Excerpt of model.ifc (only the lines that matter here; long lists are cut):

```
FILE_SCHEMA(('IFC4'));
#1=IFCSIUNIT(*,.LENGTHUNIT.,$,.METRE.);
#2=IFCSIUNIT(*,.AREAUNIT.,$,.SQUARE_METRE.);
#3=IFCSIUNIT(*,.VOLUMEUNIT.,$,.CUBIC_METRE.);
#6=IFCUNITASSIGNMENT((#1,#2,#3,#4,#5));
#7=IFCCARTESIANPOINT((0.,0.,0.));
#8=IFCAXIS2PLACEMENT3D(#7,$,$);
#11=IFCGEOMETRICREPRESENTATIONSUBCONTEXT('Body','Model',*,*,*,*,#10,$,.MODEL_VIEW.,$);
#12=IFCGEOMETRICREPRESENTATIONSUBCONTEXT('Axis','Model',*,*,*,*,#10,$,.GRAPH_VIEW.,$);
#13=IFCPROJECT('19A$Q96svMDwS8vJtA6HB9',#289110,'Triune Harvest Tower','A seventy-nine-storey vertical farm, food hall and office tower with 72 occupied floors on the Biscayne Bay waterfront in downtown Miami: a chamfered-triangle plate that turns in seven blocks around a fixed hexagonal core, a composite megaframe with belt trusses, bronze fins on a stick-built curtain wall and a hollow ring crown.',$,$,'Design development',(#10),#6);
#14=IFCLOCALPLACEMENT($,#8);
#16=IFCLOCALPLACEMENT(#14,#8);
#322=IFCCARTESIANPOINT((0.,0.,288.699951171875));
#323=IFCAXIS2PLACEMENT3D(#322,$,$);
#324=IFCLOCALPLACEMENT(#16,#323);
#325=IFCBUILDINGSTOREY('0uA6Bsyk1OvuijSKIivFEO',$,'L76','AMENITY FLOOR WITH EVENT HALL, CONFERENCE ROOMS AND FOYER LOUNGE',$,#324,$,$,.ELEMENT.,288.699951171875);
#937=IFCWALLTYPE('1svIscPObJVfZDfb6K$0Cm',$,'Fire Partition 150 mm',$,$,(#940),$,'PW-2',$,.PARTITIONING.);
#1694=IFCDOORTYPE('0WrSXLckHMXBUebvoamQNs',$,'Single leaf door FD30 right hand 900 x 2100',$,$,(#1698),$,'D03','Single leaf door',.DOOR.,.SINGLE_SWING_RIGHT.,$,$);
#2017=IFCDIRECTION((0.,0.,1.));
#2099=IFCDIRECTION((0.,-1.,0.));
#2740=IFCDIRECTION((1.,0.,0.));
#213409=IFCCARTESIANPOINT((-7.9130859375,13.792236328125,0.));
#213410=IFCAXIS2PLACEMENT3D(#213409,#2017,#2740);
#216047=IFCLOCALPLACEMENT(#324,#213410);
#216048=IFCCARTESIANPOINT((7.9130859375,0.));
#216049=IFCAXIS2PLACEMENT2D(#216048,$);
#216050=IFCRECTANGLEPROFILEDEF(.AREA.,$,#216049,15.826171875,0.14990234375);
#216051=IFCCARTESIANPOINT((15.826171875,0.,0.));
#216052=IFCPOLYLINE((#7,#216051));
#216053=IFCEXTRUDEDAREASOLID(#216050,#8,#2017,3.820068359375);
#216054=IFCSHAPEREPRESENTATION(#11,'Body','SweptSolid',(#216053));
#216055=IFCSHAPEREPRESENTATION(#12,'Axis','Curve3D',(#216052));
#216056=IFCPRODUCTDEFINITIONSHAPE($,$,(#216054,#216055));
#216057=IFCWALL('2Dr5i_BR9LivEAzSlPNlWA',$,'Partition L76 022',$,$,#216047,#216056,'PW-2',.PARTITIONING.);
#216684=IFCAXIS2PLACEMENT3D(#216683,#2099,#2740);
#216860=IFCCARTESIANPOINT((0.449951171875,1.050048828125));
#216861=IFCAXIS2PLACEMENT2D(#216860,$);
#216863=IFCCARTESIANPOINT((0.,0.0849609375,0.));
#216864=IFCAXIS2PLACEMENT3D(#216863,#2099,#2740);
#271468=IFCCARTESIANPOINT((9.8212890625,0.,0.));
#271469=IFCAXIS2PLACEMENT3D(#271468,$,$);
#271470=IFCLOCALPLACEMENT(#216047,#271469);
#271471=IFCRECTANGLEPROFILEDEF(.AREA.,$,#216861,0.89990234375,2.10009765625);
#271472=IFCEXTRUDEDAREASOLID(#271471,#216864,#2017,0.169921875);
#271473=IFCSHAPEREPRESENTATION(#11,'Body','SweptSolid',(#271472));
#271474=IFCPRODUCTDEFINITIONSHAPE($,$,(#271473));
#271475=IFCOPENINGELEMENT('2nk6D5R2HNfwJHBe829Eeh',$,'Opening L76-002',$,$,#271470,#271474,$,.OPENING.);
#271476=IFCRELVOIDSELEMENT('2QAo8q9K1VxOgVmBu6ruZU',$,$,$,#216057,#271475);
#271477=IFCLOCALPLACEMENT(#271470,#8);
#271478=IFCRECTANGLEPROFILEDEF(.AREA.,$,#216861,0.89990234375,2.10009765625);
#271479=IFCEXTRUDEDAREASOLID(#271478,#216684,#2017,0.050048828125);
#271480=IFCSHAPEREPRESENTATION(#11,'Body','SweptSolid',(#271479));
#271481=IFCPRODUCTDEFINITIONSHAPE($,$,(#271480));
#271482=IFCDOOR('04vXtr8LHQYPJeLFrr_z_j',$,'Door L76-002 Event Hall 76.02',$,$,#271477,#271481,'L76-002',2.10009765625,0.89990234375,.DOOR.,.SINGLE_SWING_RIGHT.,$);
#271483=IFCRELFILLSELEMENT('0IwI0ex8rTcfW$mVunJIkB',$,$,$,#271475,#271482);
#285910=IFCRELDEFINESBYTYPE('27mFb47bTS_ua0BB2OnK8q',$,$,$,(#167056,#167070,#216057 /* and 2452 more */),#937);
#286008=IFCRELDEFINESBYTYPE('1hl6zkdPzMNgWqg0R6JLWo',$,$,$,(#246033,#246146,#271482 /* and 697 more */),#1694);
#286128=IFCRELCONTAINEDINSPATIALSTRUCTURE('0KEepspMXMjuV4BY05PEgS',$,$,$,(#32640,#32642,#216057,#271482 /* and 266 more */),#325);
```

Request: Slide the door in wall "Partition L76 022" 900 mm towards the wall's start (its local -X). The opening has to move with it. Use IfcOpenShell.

```python
import ifcopenshell
import ifcopenshell.api.geometry
import ifcopenshell.util.placement
import ifcopenshell.util.unit

model = ifcopenshell.open("model.ifc")
unit_scale = ifcopenshell.util.unit.calculate_unit_scale(model)

door = model.by_id(271482)
opening = door.FillsVoids[0].RelatingOpeningElement
wall = opening.VoidsElements[0].RelatingBuildingElement

wall_matrix = ifcopenshell.util.placement.get_local_placement(wall.ObjectPlacement)
shift = wall_matrix[:3, 0] * -0.9 / unit_scale
before = ifcopenshell.util.placement.get_local_placement(door.ObjectPlacement)[:3, 3].copy()

# The door is placed relative to its opening, so it follows when the opening moves.
matrix = ifcopenshell.util.placement.get_local_placement(opening.ObjectPlacement)
matrix[:3, 3] += shift
ifcopenshell.api.geometry.edit_object_placement(
    model, product=opening, matrix=matrix, is_si=False, should_transform_children=True
)

after = ifcopenshell.util.placement.get_local_placement(door.ObjectPlacement)[:3, 3]
print("door moved by", (after - before).round(3) + 0.0)

model.write("model-out.ifc")
```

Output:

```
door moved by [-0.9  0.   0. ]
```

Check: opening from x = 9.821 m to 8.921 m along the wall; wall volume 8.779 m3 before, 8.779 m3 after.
